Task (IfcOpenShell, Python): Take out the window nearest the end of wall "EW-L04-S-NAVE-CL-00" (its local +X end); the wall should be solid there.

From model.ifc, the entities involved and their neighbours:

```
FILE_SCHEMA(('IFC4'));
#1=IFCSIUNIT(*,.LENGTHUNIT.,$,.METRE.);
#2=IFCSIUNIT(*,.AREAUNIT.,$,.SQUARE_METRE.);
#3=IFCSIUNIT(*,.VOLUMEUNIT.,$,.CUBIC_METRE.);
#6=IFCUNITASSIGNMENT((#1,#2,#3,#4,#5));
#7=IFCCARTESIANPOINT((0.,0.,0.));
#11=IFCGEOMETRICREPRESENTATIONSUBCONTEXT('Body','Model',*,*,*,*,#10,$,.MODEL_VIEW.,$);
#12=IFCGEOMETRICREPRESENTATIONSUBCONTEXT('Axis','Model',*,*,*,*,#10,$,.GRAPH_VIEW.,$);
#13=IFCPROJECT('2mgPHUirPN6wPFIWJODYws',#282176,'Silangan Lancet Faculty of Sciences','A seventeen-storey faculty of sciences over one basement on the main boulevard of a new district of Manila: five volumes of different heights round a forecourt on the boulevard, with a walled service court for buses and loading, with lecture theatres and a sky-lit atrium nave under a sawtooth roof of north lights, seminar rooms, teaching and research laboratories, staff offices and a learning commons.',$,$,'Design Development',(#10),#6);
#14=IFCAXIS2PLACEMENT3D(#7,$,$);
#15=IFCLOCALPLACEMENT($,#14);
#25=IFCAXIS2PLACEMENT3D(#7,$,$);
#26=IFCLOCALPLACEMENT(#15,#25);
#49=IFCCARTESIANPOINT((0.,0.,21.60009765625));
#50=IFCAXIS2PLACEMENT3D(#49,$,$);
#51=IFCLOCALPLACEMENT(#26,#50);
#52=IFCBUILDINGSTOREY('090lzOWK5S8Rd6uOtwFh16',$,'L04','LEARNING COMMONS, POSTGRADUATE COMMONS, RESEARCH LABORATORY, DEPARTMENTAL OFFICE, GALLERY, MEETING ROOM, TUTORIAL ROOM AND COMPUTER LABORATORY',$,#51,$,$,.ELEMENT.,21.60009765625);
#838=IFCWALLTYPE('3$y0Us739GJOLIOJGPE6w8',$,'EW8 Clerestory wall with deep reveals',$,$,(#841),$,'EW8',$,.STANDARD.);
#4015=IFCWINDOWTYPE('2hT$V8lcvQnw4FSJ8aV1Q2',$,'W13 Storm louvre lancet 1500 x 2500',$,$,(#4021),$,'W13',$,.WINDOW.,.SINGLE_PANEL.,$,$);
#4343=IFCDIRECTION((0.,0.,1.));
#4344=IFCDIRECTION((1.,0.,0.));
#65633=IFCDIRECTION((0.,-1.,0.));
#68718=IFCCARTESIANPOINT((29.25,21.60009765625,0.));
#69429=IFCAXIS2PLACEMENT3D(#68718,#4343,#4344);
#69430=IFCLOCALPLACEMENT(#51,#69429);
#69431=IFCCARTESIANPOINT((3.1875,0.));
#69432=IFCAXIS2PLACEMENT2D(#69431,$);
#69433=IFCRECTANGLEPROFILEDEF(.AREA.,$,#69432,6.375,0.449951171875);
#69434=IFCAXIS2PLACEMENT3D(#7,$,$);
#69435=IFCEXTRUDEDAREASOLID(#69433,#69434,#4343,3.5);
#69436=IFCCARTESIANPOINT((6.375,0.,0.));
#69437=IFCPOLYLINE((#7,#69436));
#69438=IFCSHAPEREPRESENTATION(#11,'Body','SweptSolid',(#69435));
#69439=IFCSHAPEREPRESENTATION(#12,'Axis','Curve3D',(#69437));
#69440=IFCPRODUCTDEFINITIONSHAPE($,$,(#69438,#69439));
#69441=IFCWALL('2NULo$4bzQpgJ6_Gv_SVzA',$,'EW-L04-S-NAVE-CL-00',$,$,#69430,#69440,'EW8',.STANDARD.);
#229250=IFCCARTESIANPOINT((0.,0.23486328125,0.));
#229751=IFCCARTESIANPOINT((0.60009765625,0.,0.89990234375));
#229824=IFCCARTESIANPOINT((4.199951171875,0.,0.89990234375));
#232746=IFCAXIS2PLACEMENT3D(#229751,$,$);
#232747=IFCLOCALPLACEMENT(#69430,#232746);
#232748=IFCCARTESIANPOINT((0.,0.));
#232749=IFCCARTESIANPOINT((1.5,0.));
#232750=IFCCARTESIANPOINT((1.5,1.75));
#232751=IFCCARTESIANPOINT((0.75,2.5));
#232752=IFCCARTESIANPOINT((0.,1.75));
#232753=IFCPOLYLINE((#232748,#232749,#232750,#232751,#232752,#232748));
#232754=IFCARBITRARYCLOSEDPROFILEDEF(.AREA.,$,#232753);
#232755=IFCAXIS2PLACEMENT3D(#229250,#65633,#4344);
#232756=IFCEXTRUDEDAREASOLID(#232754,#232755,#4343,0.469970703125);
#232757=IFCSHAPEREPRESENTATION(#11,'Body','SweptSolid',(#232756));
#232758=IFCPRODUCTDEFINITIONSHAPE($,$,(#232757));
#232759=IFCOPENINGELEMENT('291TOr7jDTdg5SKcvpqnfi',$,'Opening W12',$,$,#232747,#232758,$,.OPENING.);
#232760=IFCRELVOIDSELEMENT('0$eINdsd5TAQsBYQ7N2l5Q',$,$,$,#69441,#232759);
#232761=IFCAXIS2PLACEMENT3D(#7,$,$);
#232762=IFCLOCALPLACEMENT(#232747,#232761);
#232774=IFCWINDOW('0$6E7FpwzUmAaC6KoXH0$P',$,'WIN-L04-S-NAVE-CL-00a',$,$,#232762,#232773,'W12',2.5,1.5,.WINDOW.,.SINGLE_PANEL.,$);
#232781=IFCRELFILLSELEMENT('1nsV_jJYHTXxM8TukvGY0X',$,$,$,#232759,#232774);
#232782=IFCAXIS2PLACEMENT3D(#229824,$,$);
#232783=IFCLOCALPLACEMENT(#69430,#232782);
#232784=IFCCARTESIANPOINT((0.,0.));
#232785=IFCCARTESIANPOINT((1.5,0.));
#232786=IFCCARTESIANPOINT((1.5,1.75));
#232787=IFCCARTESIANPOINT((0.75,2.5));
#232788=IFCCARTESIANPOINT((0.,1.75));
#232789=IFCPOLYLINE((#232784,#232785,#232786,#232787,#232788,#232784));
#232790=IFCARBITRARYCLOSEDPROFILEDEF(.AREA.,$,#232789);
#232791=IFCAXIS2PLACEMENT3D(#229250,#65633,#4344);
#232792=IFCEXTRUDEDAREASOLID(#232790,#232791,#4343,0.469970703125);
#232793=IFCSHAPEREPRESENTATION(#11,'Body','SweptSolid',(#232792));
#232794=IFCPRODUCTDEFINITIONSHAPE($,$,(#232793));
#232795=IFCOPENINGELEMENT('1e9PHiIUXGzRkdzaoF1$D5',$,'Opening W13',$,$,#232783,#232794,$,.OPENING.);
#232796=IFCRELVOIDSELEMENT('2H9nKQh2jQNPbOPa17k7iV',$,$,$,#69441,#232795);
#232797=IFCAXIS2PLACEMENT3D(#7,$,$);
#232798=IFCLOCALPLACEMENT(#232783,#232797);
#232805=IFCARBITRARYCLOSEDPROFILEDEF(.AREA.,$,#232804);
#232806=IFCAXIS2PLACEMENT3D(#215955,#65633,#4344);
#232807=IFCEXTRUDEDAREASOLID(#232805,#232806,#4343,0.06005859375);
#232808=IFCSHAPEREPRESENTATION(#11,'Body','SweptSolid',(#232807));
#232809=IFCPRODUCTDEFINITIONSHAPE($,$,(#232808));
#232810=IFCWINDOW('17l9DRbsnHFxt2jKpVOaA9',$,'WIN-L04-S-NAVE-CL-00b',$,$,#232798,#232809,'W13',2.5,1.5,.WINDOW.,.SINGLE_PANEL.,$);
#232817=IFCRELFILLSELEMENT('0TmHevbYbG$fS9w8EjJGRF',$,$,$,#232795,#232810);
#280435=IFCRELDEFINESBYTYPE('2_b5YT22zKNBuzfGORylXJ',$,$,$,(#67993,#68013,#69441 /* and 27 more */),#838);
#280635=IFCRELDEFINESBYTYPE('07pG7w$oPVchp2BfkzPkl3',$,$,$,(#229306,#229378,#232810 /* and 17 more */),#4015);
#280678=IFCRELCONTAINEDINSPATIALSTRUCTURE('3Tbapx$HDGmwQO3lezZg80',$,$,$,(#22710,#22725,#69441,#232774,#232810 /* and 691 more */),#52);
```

```python
import ifcopenshell
import ifcopenshell.api.feature
import ifcopenshell.api.root
import ifcopenshell.geom
import ifcopenshell.util.shape

model = ifcopenshell.open("model.ifc")
settings = ifcopenshell.geom.settings()


def volume(element):
    """Net volume in cubic metres, openings subtracted."""
    shape = ifcopenshell.geom.create_shape(settings, element)
    return ifcopenshell.util.shape.get_volume(shape.geometry)


window = model.by_guid("17l9DRbsnHFxt2jKpVOaA9")
opening = window.FillsVoids[0].RelatingOpeningElement
wall = opening.VoidsElements[0].RelatingBuildingElement
before = volume(wall)

ifcopenshell.api.root.remove_product(model, product=window)
ifcopenshell.api.feature.remove_feature(model, feature=opening)

after = volume(wall)

print(f"wall volume {before:.3f} -> {after:.3f} m3")

model.write("model_updated.ifc")
```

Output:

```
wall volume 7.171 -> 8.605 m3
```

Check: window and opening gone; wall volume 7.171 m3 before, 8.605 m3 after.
